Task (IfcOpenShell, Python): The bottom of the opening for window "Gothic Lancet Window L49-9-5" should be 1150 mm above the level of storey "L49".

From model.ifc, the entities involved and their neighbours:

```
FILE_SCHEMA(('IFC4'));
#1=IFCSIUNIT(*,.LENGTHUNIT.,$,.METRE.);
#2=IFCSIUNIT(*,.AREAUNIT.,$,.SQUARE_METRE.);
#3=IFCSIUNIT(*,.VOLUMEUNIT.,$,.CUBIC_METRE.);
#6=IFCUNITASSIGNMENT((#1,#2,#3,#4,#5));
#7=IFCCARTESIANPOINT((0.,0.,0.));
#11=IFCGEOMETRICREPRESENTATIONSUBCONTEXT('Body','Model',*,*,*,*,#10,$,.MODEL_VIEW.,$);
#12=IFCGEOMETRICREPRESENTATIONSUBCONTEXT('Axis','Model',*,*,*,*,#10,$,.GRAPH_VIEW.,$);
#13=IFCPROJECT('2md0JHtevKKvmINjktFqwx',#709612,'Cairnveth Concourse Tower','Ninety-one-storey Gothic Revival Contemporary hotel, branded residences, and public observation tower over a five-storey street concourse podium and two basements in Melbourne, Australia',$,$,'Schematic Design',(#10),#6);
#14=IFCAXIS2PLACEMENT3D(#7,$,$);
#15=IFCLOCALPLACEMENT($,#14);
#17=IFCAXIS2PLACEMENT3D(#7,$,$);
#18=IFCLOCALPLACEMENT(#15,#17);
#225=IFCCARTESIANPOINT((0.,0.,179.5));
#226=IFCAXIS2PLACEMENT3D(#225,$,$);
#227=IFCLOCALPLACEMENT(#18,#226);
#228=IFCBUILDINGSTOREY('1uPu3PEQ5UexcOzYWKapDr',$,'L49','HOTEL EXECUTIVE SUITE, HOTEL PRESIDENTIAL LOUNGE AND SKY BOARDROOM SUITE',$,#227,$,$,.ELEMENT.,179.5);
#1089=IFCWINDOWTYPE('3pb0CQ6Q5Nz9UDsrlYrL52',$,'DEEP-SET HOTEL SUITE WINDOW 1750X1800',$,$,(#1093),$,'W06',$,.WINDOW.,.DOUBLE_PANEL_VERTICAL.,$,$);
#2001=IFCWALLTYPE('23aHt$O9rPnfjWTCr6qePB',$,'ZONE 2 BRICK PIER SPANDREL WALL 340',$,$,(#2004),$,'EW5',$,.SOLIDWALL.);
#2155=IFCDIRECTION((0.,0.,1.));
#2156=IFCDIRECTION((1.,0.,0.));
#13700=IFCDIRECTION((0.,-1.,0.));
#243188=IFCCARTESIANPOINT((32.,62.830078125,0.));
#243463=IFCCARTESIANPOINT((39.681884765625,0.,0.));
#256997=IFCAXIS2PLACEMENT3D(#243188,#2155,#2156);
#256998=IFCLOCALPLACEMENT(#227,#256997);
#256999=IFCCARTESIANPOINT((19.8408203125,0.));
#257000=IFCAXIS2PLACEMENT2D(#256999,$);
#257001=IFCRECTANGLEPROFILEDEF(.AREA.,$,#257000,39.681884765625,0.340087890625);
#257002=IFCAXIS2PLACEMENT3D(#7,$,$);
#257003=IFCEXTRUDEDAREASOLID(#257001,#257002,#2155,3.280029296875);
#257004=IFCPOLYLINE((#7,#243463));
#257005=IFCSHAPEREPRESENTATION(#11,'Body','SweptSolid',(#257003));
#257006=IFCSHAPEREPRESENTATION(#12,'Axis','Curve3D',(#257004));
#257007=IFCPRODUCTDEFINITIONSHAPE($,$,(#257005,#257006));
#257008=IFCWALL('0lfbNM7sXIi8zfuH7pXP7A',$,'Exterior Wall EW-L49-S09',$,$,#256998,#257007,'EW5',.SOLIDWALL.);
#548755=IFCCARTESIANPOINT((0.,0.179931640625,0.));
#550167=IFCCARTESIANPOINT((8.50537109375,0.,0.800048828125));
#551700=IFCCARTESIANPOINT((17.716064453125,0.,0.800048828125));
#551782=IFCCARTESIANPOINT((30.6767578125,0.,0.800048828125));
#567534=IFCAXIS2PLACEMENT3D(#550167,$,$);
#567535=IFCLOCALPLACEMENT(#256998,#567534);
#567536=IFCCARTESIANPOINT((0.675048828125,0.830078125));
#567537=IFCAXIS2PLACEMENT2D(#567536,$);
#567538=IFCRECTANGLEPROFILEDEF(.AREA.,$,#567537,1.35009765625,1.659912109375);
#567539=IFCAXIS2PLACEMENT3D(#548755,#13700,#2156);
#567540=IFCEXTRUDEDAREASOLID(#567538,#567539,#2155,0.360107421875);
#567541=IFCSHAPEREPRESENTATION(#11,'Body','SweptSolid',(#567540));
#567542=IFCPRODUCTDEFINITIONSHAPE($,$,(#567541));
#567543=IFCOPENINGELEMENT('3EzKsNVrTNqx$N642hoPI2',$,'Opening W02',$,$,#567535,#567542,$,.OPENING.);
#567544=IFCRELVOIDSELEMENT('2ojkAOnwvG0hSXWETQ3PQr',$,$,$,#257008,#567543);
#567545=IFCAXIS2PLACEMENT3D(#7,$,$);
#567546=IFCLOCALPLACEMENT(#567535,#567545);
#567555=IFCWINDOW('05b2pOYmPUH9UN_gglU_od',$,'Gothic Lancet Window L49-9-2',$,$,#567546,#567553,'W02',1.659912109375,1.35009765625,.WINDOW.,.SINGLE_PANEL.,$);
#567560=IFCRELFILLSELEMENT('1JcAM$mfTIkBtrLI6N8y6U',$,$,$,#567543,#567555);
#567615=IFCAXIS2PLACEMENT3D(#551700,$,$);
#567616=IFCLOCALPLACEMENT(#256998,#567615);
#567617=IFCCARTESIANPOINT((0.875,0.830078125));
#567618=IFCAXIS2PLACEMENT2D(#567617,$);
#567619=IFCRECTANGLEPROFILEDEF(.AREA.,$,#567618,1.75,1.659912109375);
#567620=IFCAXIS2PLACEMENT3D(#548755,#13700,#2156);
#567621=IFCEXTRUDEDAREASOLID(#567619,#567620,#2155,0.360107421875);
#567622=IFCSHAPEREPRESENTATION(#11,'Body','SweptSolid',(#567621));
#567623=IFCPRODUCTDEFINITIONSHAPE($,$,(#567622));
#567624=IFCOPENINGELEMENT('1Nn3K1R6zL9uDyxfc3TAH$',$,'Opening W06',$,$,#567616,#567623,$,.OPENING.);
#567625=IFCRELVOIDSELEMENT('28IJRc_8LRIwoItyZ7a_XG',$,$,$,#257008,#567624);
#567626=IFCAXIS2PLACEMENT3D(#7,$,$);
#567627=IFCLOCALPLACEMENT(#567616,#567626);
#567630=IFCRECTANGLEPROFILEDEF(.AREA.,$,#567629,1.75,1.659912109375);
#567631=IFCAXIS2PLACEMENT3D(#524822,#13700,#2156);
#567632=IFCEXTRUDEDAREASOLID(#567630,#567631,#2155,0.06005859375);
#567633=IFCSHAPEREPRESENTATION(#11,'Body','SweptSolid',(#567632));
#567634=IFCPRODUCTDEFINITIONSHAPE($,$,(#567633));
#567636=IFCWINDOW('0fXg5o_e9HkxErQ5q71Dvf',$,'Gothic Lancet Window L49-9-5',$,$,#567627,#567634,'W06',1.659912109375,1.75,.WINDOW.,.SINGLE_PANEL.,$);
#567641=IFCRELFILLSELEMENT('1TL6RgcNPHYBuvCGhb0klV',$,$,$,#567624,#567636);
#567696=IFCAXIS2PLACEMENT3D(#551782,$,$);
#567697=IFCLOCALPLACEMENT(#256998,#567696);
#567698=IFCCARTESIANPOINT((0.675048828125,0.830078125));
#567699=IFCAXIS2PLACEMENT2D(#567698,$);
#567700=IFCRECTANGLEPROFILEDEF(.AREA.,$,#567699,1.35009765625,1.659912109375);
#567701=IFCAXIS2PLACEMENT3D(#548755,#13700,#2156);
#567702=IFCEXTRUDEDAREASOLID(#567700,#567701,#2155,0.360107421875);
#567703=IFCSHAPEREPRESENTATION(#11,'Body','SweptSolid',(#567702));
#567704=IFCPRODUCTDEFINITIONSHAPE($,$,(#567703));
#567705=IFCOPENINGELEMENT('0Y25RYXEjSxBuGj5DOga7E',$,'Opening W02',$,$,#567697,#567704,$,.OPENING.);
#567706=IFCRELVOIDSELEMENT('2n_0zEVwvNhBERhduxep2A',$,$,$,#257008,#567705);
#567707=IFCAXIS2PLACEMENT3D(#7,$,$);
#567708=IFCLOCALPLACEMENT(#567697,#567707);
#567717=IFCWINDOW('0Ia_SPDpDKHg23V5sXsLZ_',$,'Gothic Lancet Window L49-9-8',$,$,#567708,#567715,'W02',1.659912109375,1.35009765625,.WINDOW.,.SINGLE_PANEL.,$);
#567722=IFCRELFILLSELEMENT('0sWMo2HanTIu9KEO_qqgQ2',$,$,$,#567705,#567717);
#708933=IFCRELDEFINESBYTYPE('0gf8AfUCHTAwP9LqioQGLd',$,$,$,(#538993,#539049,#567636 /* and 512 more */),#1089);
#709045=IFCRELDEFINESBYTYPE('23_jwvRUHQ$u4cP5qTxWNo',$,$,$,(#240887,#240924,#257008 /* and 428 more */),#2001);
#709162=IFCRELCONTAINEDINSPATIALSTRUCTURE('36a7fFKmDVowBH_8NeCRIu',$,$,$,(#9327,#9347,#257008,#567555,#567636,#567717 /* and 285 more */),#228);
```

```python
import numpy as np
import ifcopenshell
import ifcopenshell.api.geometry
import ifcopenshell.geom
import ifcopenshell.util.element
import ifcopenshell.util.placement
import ifcopenshell.util.shape
import ifcopenshell.util.unit

model = ifcopenshell.open("model.ifc")
unit_scale = ifcopenshell.util.unit.calculate_unit_scale(model)

window = model.by_guid("0fXg5o_e9HkxErQ5q71Dvf")
opening = window.FillsVoids[0].RelatingOpeningElement
storey = ifcopenshell.util.element.get_container(window, ifc_class="IfcBuildingStorey")
level = ifcopenshell.util.placement.get_local_placement(storey.ObjectPlacement)[2, 3]

# The opening's origin need not be at the sill, so measure its lowest point.
shape = ifcopenshell.geom.create_shape(ifcopenshell.geom.settings(), opening)
bottom = ifcopenshell.util.shape.get_shape_bottom_elevation(shape, shape.geometry) / unit_scale
dz = level + 1.15 - bottom

shift = np.array([0.0, 0.0, dz])
# The window is placed relative to its opening, so it follows when the opening moves.
matrix = ifcopenshell.util.placement.get_local_placement(opening.ObjectPlacement)
matrix[:3, 3] += shift
ifcopenshell.api.geometry.edit_object_placement(
    model, product=opening, matrix=matrix, is_si=False, should_transform_children=True
)

print(f"moved by {dz * unit_scale:+.3f} m")

model.write("model_updated.ifc")
```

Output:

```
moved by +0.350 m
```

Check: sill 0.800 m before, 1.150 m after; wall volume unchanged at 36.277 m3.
